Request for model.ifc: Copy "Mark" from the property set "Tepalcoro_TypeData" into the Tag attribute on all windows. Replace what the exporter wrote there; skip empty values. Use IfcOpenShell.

First a look at what the model holds.

```python
import ifcopenshell
import ifcopenshell.util.element

model = ifcopenshell.open("model.ifc")
print(model.schema)
windows = model.by_type("IfcWindow")
print(len(windows), "windows")
for e in windows[:8]:
    source = ifcopenshell.util.element.get_pset(e, "Tepalcoro_TypeData", "Mark")
    target = e.Tag
    print(e.id(), repr(source), repr(target), sep=" | ")
```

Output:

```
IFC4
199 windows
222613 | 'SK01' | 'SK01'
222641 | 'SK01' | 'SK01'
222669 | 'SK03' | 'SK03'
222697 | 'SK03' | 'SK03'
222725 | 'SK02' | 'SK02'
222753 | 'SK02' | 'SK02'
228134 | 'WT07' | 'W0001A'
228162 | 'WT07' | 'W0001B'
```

```python
import ifcopenshell
import ifcopenshell.util.element

model = ifcopenshell.open("model.ifc")

count = 0
for e in model.by_type("IfcWindow"):
    value = ifcopenshell.util.element.get_pset(e, "Tepalcoro_TypeData", "Mark")
    current = e.Tag
    if not value or not value.strip() or current == value:
        continue
    e.Tag = value
    count += 1

print(count, "windows updated")

model.write("model_edited.ifc")
```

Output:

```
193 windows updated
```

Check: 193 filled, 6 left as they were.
